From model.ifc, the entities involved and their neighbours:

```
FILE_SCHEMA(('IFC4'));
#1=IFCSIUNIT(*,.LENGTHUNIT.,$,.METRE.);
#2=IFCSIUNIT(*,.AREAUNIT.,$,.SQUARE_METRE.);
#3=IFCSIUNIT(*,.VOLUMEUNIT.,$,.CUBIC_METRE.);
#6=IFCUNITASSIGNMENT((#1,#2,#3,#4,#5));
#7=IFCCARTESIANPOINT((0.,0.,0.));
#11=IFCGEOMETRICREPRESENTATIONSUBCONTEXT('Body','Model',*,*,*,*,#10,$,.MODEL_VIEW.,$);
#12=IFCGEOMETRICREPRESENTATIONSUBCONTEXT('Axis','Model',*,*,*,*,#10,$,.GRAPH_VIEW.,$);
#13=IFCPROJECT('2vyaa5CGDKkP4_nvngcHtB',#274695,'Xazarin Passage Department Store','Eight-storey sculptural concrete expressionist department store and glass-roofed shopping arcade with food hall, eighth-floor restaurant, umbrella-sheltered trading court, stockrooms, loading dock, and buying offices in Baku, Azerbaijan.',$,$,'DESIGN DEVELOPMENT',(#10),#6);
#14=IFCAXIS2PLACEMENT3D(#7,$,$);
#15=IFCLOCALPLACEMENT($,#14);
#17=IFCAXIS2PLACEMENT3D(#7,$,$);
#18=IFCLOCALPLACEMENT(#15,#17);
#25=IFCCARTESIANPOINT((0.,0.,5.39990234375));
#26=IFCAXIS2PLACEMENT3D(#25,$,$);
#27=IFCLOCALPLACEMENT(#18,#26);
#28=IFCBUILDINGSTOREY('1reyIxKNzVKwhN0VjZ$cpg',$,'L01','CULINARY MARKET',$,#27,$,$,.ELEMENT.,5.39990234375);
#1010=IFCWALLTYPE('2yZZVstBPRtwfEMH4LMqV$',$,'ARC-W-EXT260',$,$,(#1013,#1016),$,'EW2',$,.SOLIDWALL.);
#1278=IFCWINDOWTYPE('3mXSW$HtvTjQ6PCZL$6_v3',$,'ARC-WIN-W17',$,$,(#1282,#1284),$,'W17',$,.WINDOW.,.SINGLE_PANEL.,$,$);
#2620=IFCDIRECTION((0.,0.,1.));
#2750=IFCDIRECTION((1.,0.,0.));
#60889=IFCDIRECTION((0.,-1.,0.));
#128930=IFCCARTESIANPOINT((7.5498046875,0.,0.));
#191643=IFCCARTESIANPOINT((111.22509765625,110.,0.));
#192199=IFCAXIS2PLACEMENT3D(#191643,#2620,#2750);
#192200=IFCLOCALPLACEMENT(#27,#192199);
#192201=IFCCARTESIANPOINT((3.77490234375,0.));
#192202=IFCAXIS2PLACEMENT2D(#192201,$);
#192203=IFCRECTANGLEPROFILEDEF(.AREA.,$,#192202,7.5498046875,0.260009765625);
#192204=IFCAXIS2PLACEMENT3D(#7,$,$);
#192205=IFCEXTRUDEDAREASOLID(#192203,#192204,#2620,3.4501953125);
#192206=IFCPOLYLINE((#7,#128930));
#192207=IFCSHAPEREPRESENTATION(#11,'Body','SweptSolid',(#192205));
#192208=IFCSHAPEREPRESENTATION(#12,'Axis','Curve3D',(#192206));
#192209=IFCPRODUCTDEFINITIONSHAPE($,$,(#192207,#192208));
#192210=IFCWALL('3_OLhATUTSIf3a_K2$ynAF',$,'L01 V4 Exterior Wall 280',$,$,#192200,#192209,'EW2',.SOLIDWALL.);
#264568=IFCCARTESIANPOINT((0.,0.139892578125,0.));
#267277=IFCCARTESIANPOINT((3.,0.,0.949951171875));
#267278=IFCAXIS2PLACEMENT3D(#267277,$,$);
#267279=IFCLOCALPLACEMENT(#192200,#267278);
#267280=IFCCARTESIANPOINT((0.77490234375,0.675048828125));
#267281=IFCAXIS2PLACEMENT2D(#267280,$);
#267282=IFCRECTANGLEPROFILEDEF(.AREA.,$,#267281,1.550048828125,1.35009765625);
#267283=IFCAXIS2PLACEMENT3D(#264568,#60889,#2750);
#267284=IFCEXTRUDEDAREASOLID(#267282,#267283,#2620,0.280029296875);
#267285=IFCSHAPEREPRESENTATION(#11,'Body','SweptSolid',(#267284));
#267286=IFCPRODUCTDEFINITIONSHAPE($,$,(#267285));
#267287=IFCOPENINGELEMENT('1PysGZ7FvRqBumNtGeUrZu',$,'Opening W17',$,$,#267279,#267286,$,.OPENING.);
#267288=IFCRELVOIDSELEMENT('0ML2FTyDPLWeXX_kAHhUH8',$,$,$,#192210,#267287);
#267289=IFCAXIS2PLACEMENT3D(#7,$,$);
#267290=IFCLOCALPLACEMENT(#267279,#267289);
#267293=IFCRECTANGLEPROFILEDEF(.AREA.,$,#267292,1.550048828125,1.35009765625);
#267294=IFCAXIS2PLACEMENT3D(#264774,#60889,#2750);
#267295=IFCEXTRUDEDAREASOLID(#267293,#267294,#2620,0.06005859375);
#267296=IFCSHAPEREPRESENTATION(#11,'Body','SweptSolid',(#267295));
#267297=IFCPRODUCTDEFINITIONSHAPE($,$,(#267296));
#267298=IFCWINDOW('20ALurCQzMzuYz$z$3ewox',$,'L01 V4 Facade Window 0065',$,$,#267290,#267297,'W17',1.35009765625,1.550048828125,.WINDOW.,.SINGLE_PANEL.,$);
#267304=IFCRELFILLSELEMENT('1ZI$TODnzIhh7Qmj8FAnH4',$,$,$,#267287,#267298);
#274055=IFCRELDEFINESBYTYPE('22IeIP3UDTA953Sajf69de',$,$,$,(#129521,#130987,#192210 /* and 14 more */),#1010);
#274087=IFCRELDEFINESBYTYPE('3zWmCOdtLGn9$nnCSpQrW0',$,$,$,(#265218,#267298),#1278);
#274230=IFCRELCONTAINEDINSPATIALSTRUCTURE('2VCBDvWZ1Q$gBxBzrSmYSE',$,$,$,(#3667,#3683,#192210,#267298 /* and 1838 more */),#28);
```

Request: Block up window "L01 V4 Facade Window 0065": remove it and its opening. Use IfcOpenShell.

```python
import ifcopenshell
import ifcopenshell.api.feature
import ifcopenshell.api.root
import ifcopenshell.geom
import ifcopenshell.util.shape

model = ifcopenshell.open("model.ifc")
settings = ifcopenshell.geom.settings()


def volume(element):
    """Net volume in cubic metres, openings subtracted."""
    shape = ifcopenshell.geom.create_shape(settings, element)
    return ifcopenshell.util.shape.get_volume(shape.geometry)


window = model.by_guid("20ALurCQzMzuYz$z$3ewox")
opening = window.FillsVoids[0].RelatingOpeningElement
wall = opening.VoidsElements[0].RelatingBuildingElement
before = volume(wall)

ifcopenshell.api.root.remove_product(model, product=window)
ifcopenshell.api.feature.remove_feature(model, feature=opening)

after = volume(wall)

print(f"wall volume {before:.3f} -> {after:.3f} m3")

model.write("model_v2.ifc")
```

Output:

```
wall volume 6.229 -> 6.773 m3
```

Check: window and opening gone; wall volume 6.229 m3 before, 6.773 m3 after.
